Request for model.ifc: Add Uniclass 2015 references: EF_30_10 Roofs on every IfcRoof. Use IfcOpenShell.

First a look at what the model holds.

```python
import ifcopenshell

model = ifcopenshell.open("model.ifc")
print(model.schema)
print("classifications:", [c.Name for c in model.by_type("IfcClassification")])
for ifc_class in ("IfcDoor", "IfcRoof", "IfcStair", "IfcWall", "IfcWindow"):
    print(ifc_class, len(model.by_type(ifc_class)))
```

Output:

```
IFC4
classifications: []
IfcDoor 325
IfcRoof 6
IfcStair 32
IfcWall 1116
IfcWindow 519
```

```python
import ifcopenshell
import ifcopenshell.api.classification

model = ifcopenshell.open("model.ifc")

system = ifcopenshell.api.classification.add_classification(model, classification="Uniclass 2015")

codes = {
    "IfcRoof": ("EF_30_10", "Roofs"),
}
for ifc_class, (code, name) in codes.items():
    products = model.by_type(ifc_class)
    ifcopenshell.api.classification.add_reference(
        model, products=products, classification=system, identification=code, name=name
    )
    print(code, len(products))

model.write("model-out.ifc")
```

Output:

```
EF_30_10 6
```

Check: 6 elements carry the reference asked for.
